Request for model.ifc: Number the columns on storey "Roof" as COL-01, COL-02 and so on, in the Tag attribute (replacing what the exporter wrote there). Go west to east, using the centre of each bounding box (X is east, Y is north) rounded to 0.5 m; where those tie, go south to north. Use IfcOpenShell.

First a look at what the model holds.

```python
import ifcopenshell
import ifcopenshell.util.element
import ifcopenshell.util.placement

model = ifcopenshell.open("model.ifc")
print(model.schema)
storey = next(s for s in model.by_type("IfcBuildingStorey") if s.Name == "Roof")
columns = [e for e in ifcopenshell.util.element.get_decomposition(storey) if e.is_a("IfcColumn")]
for e in sorted(columns, key=lambda e: e.id()):
    origin = ifcopenshell.util.placement.get_local_placement(e.ObjectPlacement)[:3, 3]
    print(e.id(), e.Tag, e.Name, origin.round(2) + 0.0, sep=" | ")
```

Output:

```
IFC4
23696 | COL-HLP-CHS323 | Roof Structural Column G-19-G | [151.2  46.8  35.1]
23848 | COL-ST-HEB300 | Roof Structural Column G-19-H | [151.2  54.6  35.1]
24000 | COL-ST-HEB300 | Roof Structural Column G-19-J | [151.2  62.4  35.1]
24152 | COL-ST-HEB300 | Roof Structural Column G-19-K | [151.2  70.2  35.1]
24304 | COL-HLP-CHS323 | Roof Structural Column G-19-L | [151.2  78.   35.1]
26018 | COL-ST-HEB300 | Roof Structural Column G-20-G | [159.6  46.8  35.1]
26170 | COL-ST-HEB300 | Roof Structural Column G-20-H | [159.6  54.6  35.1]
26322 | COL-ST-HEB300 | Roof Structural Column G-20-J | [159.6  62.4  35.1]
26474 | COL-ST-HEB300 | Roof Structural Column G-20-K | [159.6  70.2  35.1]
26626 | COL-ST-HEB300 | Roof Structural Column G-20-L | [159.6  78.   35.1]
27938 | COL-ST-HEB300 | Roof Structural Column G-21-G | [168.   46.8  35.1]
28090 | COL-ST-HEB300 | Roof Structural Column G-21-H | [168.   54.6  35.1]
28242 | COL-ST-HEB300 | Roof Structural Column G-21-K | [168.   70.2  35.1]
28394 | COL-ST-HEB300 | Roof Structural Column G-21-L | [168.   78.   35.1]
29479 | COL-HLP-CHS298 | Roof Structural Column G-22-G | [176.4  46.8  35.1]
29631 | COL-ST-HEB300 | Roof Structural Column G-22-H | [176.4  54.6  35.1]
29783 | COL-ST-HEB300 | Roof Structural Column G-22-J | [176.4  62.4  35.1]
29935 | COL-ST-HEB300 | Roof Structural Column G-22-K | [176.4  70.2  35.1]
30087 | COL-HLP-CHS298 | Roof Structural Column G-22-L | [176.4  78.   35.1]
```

```python
import ifcopenshell
import ifcopenshell.geom
import ifcopenshell.util.element
import ifcopenshell.util.shape

model = ifcopenshell.open("model.ifc")
settings = ifcopenshell.geom.settings()
settings.set("use-world-coords", True)


def centre(element):
    shape = ifcopenshell.geom.create_shape(settings, element)
    return ifcopenshell.util.shape.get_bbox_centroid(shape.geometry)


storey = next(s for s in model.by_type("IfcBuildingStorey") if s.Name == "Roof")
columns = [e for e in ifcopenshell.util.element.get_decomposition(storey) if e.is_a("IfcColumn")]

# Insertion points can sit at a corner or the storey origin, so sort by the geometry (in metres).
centres = {e: centre(e) for e in columns}
columns.sort(key=lambda e: (round(centres[e][0] / 0.5), centres[e][1]))

for i, e in enumerate(columns, start=1):
    number = f"COL-{i:02d}"
    e.Tag = number
    print(e.id(), number)

model.write("model_edited.ifc")
```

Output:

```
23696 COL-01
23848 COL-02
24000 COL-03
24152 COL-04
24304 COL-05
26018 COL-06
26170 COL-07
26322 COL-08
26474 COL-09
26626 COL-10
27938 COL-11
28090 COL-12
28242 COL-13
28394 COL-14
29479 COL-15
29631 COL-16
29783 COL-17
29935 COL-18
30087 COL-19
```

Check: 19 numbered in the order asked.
